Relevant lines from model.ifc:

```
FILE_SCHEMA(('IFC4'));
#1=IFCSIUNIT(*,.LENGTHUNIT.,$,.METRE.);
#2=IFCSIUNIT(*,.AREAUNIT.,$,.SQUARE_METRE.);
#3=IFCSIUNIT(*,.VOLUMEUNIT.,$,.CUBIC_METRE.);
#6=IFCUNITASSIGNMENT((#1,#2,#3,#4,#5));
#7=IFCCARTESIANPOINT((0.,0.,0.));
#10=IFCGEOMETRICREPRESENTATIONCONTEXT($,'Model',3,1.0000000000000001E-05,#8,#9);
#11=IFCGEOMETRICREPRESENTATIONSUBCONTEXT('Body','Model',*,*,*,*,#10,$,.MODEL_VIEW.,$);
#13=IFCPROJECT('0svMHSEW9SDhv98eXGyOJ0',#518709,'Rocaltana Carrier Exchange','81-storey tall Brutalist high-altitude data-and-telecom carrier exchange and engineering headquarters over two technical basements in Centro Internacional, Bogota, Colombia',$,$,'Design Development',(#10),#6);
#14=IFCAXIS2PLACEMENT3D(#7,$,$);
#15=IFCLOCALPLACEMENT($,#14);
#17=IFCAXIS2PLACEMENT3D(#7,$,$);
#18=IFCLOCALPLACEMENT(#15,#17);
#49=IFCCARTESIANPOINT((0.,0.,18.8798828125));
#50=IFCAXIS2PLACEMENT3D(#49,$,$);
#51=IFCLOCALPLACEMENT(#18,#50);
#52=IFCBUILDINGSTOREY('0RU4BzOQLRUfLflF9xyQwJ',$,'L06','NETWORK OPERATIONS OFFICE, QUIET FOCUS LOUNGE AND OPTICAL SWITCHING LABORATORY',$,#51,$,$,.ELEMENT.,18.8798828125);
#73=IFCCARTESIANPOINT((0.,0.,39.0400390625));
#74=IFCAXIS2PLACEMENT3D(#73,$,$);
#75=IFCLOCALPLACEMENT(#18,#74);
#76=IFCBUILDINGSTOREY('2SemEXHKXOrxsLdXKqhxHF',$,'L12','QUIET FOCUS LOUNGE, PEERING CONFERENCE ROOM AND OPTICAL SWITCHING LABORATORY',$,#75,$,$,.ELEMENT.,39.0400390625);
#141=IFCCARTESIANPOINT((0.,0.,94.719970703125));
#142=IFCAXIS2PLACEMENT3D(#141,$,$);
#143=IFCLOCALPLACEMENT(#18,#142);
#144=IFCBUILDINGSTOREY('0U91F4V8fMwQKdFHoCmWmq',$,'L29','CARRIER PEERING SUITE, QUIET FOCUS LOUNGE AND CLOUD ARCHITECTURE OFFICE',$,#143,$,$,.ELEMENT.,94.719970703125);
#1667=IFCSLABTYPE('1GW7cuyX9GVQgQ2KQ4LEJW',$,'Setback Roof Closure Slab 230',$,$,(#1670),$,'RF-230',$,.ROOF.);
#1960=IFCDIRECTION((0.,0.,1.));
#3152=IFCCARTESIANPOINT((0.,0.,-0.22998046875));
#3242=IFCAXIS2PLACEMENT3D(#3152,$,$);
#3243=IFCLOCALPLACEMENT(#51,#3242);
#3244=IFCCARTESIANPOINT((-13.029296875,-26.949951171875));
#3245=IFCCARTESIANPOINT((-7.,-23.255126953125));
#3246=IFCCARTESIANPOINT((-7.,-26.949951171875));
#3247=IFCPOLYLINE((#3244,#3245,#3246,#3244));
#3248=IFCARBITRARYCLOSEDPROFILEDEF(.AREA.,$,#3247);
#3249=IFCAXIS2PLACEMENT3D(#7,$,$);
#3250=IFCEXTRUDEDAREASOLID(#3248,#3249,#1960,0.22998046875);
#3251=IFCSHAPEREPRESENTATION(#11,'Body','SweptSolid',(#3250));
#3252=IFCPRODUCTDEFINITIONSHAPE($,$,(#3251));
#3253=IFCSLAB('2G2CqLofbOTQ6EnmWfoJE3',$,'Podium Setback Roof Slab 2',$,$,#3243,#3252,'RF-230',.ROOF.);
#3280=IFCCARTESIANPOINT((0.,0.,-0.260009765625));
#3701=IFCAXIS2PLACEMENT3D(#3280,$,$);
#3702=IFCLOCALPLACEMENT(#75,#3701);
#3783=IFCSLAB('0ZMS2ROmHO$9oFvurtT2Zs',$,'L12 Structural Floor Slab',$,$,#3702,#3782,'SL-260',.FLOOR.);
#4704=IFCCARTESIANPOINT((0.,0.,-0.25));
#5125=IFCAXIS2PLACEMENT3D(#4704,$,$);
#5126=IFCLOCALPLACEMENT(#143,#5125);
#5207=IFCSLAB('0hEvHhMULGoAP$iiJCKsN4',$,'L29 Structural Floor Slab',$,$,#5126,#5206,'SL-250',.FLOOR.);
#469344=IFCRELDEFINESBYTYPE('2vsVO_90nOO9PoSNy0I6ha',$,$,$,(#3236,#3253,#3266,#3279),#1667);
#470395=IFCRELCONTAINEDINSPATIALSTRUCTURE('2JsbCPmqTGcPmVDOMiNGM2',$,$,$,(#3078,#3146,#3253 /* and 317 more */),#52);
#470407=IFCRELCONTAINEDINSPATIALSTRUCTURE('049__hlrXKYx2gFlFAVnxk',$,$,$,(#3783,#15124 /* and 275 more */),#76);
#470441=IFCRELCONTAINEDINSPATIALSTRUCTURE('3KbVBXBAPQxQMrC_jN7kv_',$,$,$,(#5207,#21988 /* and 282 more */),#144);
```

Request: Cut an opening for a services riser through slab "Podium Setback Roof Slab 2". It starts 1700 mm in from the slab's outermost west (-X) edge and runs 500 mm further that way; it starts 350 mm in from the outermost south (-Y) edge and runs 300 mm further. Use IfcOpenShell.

```python
import numpy as np
import ifcopenshell
import ifcopenshell.api.feature
import ifcopenshell.api.geometry
import ifcopenshell.api.root
import ifcopenshell.geom
import ifcopenshell.util.placement
import ifcopenshell.util.representation
import ifcopenshell.util.shape
import ifcopenshell.util.unit

model = ifcopenshell.open("model.ifc")
unit_scale = ifcopenshell.util.unit.calculate_unit_scale(model)
settings = ifcopenshell.geom.settings()


def volume(element):
    """Net volume in cubic metres, openings subtracted."""
    shape = ifcopenshell.geom.create_shape(settings, element)
    return ifcopenshell.util.shape.get_volume(shape.geometry)


slab = model.by_guid("2G2CqLofbOTQ6EnmWfoJE3")
before = volume(slab)

# Extent in the slab's own axes, in metres. The edges named are its -X and -Y sides.
slab_shape = ifcopenshell.geom.create_shape(settings, slab)
vertices = ifcopenshell.util.shape.get_vertices(slab_shape.geometry)
x_min, y_min, bottom = vertices.min(axis=0)
top = vertices[:, 2].max()

opening = ifcopenshell.api.root.create_entity(model, ifc_class="IfcOpeningElement", name="Services riser opening", predefined_type="OPENING")
context = ifcopenshell.util.representation.get_context(model, "Model", "Body", "MODEL_VIEW")
width, depth = 0.5, 0.3
outline = [(0.0, 0.0), (width, 0.0), (width, depth), (0.0, depth), (0.0, 0.0)]
# Overshoot both faces by 50 mm so the cut is clean.
shape = ifcopenshell.api.geometry.add_slab_representation(
    model, context=context, depth=top - bottom + 0.1, polyline=outline
)
ifcopenshell.api.geometry.assign_representation(model, product=opening, representation=shape)

matrix = ifcopenshell.util.placement.get_local_placement(slab.ObjectPlacement)
matrix[:, 3] = matrix @ np.append(np.array([x_min + 1.7, y_min + 0.35, bottom - 0.05]) / unit_scale, 1.0)
ifcopenshell.api.geometry.edit_object_placement(model, product=opening, matrix=matrix, is_si=False)
ifcopenshell.api.feature.add_feature(model, feature=opening, element=slab)

after = volume(slab)

print(f"slab volume {before:.3f} -> {after:.3f} m3")

model.write("model_edited.ifc")
```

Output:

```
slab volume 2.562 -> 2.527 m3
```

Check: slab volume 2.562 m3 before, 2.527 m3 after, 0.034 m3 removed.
